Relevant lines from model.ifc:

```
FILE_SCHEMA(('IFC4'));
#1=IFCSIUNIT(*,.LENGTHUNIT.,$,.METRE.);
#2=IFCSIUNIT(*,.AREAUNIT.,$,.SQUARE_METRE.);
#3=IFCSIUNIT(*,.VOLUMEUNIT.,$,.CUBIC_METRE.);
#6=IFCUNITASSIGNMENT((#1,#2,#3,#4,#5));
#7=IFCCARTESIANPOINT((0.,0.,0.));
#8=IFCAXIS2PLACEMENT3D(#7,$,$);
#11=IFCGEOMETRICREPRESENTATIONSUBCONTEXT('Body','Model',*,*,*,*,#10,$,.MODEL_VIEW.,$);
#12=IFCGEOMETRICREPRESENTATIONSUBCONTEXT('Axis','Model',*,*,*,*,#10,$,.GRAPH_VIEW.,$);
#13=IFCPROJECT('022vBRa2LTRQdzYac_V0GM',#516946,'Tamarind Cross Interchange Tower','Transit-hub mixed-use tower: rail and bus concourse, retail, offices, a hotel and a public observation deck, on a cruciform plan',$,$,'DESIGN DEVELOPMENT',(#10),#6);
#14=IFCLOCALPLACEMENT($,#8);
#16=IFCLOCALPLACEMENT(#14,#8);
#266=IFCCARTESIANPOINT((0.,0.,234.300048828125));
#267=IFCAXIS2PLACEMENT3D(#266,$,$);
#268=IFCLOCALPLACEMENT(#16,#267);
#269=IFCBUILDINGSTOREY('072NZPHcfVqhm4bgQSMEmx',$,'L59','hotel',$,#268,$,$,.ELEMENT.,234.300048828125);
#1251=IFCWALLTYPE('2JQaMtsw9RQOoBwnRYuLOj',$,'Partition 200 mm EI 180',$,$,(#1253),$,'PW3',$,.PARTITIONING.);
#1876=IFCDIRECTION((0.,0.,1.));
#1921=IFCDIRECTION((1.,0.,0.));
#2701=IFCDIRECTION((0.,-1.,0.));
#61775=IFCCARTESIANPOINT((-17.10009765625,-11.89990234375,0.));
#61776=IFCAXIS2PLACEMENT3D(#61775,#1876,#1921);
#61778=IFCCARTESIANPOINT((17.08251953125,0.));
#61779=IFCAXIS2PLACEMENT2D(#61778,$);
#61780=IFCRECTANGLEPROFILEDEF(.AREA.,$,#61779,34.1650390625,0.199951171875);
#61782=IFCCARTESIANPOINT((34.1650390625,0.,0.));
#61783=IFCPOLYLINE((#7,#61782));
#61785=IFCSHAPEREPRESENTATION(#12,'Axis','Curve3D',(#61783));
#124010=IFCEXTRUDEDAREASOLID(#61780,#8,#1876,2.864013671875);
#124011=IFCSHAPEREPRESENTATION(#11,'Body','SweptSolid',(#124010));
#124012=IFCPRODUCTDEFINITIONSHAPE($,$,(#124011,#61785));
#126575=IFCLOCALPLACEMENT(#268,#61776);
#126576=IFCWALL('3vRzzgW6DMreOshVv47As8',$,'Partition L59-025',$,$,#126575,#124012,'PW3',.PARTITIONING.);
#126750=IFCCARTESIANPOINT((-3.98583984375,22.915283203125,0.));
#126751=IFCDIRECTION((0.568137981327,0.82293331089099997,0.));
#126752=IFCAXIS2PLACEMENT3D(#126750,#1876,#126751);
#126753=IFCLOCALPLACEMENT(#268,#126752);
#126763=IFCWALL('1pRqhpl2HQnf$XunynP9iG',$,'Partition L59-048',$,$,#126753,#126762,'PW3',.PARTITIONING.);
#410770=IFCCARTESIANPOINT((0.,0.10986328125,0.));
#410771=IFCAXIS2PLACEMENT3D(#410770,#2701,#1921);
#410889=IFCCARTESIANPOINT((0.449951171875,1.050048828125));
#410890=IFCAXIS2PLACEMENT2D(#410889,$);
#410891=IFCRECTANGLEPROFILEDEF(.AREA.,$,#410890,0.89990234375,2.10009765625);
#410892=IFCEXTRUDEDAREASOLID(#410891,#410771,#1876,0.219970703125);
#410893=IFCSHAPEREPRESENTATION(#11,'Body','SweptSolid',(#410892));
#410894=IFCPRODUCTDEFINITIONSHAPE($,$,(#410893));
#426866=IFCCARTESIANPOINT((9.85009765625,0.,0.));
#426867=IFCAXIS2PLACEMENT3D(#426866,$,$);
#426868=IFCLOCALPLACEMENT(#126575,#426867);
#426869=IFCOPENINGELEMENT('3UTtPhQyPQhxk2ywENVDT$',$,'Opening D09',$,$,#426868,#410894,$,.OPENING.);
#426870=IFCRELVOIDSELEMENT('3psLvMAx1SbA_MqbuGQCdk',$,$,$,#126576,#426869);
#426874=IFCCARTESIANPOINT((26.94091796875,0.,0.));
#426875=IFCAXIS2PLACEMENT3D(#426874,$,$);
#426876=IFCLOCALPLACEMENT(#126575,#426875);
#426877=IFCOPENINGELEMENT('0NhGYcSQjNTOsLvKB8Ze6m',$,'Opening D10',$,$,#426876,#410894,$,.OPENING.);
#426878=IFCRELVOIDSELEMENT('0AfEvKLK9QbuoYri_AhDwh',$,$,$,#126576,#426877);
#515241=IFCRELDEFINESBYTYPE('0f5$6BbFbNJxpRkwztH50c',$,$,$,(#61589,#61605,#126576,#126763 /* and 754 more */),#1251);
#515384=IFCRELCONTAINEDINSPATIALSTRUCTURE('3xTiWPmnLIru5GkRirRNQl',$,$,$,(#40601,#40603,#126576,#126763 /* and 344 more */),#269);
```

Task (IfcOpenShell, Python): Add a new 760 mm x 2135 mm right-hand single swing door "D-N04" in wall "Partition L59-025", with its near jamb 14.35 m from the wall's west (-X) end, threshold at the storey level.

```python
import numpy as np
import ifcopenshell
import ifcopenshell.api.feature
import ifcopenshell.api.geometry
import ifcopenshell.api.root
import ifcopenshell.api.spatial
import ifcopenshell.geom
import ifcopenshell.util.element
import ifcopenshell.util.placement
import ifcopenshell.util.representation
import ifcopenshell.util.shape
import ifcopenshell.util.unit

model = ifcopenshell.open("model.ifc")
unit_scale = ifcopenshell.util.unit.calculate_unit_scale(model)
settings = ifcopenshell.geom.settings()


def volume(element):
    """Net volume in cubic metres, openings subtracted."""
    shape = ifcopenshell.geom.create_shape(settings, element)
    return ifcopenshell.util.shape.get_volume(shape.geometry)


wall = model.by_guid("3vRzzgW6DMreOshVv47As8")
storey = ifcopenshell.util.element.get_container(wall, ifc_class="IfcBuildingStorey")
context = ifcopenshell.util.representation.get_context(model, "Model", "Body", "MODEL_VIEW")
before = volume(wall)

width, height, from_end, sill = 0.76, 2.135, 14.35, 0.0  # metres

# The wall runs along its own X axis, and the end named is its -X end.
wall_shape = ifcopenshell.geom.create_shape(settings, wall)
x, y, z = ifcopenshell.util.shape.get_vertices(wall_shape.geometry).T
start = x.min() + from_end
face, thickness = float(y.min()), float(y.max() - y.min())
wall_matrix = ifcopenshell.util.placement.get_local_placement(wall.ObjectPlacement)
level = ifcopenshell.util.placement.get_local_placement(storey.ObjectPlacement)[2, 3]


def in_wall(x, y):
    """Placement at x, y metres in the wall's axes, at sill height."""
    matrix = wall_matrix.copy()
    matrix[:, 3] = wall_matrix @ np.array([x / unit_scale, y / unit_scale, 0.0, 1.0])
    matrix[2, 3] = level + sill / unit_scale
    return matrix


# Opening: a box that overshoots both wall faces by 50 mm.
opening = ifcopenshell.api.root.create_entity(model, ifc_class="IfcOpeningElement", predefined_type="OPENING")
box = ifcopenshell.api.geometry.add_wall_representation(
    model, context=context, length=width, height=height, thickness=thickness + 0.1
)
ifcopenshell.api.geometry.assign_representation(model, product=opening, representation=box)
ifcopenshell.api.geometry.edit_object_placement(model, product=opening, matrix=in_wall(start, face - 0.05), is_si=False)
ifcopenshell.api.feature.add_feature(model, feature=opening, element=wall)

door = ifcopenshell.api.root.create_entity(model, ifc_class="IfcDoor", name="D-N04", predefined_type="DOOR")
door.OverallWidth, door.OverallHeight = width / unit_scale, height / unit_scale
door.OperationType = "SINGLE_SWING_RIGHT"
body = ifcopenshell.api.geometry.add_door_representation(
    model,
    context=context,
    overall_width=door.OverallWidth,
    overall_height=door.OverallHeight,
    operation_type="SINGLE_SWING_RIGHT",
    lining_properties={"LiningDepth": thickness / unit_scale, "ThresholdDepth": thickness / unit_scale},
)
ifcopenshell.api.geometry.assign_representation(model, product=door, representation=body)
ifcopenshell.api.spatial.assign_container(model, products=[door], relating_structure=storey)
ifcopenshell.api.feature.add_filling(model, opening=opening, element=door)

# The lining spans the wall, so the door starts at the wall face.
ifcopenshell.api.geometry.edit_object_placement(model, product=door, matrix=in_wall(start, face), is_si=False)

after = volume(wall)

print(f"wall volume {before:.3f} -> {after:.3f} m3")

model.write("model_edited.ifc")
```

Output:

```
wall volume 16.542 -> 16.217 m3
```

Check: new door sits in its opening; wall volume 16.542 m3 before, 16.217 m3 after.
